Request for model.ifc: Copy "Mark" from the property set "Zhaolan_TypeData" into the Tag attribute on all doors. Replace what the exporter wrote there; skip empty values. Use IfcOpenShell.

First a look at what the model holds.

```python
import ifcopenshell
import ifcopenshell.util.element

model = ifcopenshell.open("model.ifc")
print(model.schema)
doors = model.by_type("IfcDoor")
print(len(doors), "doors")
for e in doors[:8]:
    source = ifcopenshell.util.element.get_pset(e, "Zhaolan_TypeData", "Mark")
    target = e.Tag
    print(e.id(), repr(source), repr(target), sep=" | ")
```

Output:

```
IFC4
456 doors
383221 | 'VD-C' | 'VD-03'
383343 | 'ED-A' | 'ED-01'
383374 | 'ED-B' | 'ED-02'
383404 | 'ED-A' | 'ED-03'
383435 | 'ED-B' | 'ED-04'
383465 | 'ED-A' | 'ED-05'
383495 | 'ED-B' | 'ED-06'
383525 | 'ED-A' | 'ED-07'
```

```python
import ifcopenshell
import ifcopenshell.util.element

model = ifcopenshell.open("model.ifc")

count = 0
for e in model.by_type("IfcDoor"):
    value = ifcopenshell.util.element.get_pset(e, "Zhaolan_TypeData", "Mark")
    current = e.Tag
    if not value or not value.strip() or current == value:
        continue
    e.Tag = value
    count += 1

print(count, "doors updated")

model.write("model_updated.ifc")
```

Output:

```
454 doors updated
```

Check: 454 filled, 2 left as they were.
